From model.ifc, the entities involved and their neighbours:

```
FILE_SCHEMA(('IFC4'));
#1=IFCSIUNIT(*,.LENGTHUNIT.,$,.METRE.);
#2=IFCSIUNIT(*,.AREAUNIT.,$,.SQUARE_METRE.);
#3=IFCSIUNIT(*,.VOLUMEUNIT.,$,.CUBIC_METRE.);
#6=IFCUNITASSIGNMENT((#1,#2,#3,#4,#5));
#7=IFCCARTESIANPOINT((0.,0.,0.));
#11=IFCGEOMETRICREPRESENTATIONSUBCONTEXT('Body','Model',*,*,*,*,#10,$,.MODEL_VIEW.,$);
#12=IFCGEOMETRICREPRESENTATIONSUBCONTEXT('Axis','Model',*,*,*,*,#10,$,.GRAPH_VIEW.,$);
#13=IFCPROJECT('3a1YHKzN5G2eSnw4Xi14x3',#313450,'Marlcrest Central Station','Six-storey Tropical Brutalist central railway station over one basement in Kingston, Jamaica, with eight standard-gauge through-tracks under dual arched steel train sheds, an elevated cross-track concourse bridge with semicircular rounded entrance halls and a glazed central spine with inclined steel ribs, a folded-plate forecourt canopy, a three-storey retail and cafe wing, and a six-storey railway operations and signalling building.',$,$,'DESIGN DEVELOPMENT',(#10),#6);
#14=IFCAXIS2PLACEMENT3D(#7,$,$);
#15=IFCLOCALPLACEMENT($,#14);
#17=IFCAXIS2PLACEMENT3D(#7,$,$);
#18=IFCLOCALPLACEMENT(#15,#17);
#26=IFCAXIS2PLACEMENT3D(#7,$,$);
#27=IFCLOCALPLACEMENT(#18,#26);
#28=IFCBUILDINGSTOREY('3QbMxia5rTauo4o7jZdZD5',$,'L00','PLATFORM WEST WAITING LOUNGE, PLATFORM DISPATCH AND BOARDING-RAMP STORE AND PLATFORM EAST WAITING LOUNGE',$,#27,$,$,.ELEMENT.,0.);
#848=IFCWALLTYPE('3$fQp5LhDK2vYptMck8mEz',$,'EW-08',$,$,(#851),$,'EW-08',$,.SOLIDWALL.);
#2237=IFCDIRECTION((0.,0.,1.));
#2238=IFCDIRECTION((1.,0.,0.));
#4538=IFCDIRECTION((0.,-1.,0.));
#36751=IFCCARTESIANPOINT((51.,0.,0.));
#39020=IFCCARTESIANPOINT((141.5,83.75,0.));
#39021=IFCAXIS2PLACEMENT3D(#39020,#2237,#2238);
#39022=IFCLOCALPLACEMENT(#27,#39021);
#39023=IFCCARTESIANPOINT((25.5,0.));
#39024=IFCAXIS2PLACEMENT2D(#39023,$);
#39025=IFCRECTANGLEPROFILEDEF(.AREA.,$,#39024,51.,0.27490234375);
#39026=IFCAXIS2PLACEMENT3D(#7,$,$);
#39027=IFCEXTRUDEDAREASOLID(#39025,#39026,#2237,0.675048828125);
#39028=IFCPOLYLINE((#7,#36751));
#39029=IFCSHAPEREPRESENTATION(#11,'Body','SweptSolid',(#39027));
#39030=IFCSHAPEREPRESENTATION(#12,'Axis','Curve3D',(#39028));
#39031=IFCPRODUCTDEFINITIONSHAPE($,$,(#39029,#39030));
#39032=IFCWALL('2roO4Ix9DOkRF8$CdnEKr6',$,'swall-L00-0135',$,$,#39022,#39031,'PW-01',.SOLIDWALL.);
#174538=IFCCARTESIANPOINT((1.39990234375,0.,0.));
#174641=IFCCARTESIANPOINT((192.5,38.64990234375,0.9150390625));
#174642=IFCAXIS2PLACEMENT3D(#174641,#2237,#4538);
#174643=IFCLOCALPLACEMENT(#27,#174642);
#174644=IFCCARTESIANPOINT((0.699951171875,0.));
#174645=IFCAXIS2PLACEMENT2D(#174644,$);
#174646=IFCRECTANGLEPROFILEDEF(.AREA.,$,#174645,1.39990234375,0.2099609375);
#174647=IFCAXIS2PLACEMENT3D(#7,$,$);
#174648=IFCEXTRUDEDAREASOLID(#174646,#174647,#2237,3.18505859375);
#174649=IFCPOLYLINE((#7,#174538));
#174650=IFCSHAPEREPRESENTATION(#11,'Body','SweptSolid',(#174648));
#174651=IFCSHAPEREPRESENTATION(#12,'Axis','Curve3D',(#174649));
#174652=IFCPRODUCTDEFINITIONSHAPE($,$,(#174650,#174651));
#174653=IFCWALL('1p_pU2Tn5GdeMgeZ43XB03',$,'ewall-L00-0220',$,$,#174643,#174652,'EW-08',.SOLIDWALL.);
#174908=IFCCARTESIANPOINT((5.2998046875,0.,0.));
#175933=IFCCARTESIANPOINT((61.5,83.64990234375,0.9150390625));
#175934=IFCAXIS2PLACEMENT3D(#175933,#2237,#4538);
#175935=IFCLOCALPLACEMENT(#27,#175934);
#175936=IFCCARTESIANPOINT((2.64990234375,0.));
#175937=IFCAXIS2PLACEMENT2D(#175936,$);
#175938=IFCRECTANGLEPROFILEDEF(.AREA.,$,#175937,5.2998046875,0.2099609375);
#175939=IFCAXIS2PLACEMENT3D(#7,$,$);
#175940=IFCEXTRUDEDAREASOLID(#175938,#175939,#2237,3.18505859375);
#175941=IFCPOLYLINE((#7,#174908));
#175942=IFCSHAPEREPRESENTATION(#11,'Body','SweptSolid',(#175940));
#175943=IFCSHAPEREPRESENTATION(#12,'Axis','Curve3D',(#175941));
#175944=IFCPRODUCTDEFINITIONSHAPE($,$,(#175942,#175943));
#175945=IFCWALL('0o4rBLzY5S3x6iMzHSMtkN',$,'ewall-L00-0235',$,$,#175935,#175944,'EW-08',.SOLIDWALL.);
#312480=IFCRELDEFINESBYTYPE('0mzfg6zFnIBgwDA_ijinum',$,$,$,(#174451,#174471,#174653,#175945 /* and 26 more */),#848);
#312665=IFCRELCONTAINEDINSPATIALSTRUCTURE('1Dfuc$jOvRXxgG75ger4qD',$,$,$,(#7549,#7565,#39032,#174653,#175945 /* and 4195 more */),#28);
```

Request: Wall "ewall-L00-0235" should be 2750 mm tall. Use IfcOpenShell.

```python
import ifcopenshell
import ifcopenshell.geom
import ifcopenshell.util.representation
import ifcopenshell.util.shape

model = ifcopenshell.open("model.ifc")
settings = ifcopenshell.geom.settings()


def volume(element):
    """Net volume in cubic metres, openings subtracted."""
    shape = ifcopenshell.geom.create_shape(settings, element)
    return ifcopenshell.util.shape.get_volume(shape.geometry)


wall = model.by_id(175945)
before = volume(wall)

body = ifcopenshell.util.representation.get_representation(wall, "Model", "Body")
solid = body.Items[0]
old_height = solid.Depth
solid.Depth = 2.75
after = volume(wall)

print(f"height {old_height:g} -> {solid.Depth:g}, volume {before:.3f} -> {after:.3f} m3")

model.write("model-out.ifc")
```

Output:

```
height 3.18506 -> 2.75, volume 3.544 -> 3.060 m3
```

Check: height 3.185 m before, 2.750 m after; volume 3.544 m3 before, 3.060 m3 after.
